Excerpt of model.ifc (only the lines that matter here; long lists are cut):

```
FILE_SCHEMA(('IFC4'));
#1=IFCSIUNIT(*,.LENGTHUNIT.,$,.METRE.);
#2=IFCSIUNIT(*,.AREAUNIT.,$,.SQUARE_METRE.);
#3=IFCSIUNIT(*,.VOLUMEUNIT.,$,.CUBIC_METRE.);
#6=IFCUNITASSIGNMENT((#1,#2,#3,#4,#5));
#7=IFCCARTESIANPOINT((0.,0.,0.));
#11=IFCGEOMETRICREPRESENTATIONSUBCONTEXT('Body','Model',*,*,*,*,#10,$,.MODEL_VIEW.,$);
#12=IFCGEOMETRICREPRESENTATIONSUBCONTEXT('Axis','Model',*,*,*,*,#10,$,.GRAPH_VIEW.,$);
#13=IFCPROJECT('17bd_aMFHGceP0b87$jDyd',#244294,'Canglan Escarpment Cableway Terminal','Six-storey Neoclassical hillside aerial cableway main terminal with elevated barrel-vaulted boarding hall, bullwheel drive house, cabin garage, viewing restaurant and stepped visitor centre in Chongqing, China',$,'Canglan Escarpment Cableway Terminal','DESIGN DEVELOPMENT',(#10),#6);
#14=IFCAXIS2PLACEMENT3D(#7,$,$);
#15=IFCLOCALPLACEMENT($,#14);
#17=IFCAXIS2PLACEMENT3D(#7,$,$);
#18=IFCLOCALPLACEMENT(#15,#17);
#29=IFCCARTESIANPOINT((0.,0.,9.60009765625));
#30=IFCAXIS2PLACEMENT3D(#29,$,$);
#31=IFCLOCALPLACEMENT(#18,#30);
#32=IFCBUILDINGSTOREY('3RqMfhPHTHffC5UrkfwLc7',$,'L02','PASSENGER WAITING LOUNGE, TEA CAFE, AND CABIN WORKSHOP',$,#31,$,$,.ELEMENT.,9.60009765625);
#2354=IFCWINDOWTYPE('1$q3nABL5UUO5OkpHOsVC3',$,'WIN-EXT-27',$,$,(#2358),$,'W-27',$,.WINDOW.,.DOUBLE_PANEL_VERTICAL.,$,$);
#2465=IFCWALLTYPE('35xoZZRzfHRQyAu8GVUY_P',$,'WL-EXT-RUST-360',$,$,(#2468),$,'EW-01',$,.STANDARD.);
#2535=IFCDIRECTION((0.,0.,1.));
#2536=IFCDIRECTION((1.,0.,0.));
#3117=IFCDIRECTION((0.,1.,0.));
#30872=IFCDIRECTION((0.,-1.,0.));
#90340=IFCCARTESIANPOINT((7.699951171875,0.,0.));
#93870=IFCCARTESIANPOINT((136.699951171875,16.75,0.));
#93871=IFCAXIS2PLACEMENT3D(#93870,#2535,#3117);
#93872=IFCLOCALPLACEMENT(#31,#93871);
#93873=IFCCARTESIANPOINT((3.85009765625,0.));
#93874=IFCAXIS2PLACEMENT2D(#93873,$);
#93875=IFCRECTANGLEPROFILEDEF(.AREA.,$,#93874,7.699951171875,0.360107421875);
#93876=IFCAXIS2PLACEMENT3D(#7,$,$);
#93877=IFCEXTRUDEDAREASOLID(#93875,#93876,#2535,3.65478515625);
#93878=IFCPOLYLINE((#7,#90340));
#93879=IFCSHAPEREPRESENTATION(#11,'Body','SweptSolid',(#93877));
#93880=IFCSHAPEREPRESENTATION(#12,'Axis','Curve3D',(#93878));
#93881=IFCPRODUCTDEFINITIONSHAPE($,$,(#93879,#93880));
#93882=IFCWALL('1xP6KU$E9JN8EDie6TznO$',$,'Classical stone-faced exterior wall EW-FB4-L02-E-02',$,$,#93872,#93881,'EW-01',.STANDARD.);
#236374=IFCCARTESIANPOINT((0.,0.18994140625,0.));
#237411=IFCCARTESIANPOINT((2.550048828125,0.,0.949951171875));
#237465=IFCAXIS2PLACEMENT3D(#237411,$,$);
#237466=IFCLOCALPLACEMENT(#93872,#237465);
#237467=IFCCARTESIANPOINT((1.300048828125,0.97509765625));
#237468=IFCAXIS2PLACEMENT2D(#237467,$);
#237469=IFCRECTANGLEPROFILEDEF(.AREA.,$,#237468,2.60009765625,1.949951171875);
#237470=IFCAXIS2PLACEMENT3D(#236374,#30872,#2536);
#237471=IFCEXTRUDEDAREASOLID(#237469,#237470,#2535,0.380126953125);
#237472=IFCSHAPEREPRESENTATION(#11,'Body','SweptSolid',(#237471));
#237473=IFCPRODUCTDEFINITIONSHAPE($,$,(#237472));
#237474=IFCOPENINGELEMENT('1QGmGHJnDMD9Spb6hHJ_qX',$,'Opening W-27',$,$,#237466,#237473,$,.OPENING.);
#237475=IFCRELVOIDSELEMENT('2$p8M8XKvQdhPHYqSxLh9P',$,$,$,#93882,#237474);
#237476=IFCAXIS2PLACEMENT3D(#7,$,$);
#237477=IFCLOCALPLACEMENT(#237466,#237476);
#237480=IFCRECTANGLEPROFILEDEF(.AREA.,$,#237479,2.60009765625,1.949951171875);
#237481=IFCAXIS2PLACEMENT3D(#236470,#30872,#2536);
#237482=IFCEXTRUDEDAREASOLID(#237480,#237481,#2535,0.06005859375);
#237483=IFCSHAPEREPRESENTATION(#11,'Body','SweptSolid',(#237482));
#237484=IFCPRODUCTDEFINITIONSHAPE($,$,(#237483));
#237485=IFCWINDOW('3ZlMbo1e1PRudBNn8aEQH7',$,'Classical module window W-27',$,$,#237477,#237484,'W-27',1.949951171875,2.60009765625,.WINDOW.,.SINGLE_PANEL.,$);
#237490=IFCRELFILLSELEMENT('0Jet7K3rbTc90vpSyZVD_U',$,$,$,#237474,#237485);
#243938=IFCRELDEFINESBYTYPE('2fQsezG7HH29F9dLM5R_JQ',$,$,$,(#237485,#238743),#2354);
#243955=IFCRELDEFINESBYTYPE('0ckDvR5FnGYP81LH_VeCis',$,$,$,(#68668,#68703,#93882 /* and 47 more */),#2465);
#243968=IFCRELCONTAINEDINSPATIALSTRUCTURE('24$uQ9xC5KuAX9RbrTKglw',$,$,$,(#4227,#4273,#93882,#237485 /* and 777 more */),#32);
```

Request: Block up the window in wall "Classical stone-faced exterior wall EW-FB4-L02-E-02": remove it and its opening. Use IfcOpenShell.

```python
import ifcopenshell
import ifcopenshell.api.feature
import ifcopenshell.api.root
import ifcopenshell.geom
import ifcopenshell.util.shape

model = ifcopenshell.open("model.ifc")
settings = ifcopenshell.geom.settings()


def volume(element):
    """Net volume in cubic metres, openings subtracted."""
    shape = ifcopenshell.geom.create_shape(settings, element)
    return ifcopenshell.util.shape.get_volume(shape.geometry)


window = model.by_guid("3ZlMbo1e1PRudBNn8aEQH7")
opening = window.FillsVoids[0].RelatingOpeningElement
wall = opening.VoidsElements[0].RelatingBuildingElement
before = volume(wall)

ifcopenshell.api.root.remove_product(model, product=window)
ifcopenshell.api.feature.remove_feature(model, feature=opening)

after = volume(wall)

print(f"wall volume {before:.3f} -> {after:.3f} m3")

model.write("model_v2.ifc")
```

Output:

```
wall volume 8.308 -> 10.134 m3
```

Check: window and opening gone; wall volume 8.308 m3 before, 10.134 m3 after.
